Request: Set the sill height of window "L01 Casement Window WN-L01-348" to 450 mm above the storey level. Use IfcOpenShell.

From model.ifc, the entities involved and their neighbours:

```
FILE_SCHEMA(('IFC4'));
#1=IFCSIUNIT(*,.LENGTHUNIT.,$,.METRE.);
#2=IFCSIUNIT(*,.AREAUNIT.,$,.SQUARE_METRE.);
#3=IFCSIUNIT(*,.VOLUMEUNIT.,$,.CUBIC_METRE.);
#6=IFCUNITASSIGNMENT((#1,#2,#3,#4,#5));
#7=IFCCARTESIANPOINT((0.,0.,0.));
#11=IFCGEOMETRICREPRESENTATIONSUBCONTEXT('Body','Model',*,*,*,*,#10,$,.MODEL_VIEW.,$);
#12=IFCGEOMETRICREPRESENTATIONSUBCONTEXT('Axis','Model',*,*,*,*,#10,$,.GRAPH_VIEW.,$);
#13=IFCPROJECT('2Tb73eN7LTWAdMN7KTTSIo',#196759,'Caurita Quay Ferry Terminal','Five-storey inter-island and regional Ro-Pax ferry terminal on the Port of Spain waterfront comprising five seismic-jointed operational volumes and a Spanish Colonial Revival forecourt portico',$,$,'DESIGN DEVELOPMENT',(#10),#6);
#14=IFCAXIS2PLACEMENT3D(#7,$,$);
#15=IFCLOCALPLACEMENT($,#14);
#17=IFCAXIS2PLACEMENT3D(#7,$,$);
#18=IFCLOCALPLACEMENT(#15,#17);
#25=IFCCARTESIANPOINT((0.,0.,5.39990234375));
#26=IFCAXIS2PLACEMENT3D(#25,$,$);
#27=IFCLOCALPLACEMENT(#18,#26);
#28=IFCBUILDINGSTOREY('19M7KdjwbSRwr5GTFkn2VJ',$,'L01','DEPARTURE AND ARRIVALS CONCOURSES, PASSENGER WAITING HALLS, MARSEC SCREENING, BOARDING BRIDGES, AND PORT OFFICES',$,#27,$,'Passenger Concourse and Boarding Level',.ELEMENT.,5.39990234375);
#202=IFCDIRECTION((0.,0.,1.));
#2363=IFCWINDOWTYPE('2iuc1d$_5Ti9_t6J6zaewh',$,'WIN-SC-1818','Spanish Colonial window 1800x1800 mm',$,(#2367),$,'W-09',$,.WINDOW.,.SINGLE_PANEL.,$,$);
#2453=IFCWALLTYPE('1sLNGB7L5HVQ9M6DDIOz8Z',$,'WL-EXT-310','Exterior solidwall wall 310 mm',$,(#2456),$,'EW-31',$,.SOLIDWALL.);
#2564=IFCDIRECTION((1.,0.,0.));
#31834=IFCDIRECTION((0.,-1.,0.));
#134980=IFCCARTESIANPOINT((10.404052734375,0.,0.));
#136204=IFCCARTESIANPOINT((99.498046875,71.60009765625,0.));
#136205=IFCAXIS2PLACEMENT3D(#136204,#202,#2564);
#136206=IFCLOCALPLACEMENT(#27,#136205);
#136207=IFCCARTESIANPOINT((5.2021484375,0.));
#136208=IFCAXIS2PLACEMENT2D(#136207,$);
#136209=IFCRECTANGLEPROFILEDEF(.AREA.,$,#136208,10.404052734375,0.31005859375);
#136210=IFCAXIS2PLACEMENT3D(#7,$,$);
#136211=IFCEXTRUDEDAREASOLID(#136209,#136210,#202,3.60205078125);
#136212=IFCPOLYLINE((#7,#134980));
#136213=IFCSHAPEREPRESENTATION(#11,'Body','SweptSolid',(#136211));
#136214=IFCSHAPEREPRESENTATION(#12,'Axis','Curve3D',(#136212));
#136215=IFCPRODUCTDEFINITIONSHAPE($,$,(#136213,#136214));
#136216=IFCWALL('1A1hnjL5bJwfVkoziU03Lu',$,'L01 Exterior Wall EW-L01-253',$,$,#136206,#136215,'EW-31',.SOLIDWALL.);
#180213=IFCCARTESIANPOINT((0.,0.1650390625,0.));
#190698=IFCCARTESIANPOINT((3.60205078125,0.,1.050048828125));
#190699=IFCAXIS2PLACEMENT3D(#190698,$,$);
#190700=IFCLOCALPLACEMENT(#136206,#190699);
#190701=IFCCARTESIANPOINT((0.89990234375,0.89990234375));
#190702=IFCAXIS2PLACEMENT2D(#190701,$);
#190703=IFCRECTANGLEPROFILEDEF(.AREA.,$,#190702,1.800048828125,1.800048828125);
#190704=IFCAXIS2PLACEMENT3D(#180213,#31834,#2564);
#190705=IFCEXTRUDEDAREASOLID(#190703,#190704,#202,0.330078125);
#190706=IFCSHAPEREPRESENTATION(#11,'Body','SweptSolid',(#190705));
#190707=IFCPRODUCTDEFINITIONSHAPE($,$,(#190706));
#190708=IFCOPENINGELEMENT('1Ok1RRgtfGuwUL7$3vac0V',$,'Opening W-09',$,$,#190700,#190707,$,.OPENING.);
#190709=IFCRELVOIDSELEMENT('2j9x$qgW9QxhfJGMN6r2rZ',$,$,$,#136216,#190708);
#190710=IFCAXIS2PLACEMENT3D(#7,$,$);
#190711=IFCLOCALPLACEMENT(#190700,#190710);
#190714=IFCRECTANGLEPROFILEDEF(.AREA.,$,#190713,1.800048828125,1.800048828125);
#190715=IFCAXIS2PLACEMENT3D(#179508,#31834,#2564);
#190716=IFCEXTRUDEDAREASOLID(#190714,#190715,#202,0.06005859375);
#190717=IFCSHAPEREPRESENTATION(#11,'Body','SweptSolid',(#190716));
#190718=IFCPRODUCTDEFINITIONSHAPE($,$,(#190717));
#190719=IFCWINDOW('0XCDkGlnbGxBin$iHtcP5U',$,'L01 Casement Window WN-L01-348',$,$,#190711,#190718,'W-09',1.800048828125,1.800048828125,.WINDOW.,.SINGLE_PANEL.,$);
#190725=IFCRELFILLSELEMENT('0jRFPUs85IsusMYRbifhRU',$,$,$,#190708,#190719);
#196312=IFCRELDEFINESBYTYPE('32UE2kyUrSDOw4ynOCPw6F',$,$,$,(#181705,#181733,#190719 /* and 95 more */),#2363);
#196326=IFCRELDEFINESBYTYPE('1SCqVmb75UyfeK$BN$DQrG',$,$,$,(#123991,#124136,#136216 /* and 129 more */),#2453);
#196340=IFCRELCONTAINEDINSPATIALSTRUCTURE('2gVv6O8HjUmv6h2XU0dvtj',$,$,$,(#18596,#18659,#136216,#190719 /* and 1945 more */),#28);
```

```python
import numpy as np
import ifcopenshell
import ifcopenshell.api.geometry
import ifcopenshell.geom
import ifcopenshell.util.element
import ifcopenshell.util.placement
import ifcopenshell.util.shape
import ifcopenshell.util.unit

model = ifcopenshell.open("model.ifc")
unit_scale = ifcopenshell.util.unit.calculate_unit_scale(model)

window = model.by_guid("0XCDkGlnbGxBin$iHtcP5U")
opening = window.FillsVoids[0].RelatingOpeningElement
storey = ifcopenshell.util.element.get_container(window, ifc_class="IfcBuildingStorey")
level = ifcopenshell.util.placement.get_local_placement(storey.ObjectPlacement)[2, 3]

# The opening's origin need not be at the sill, so measure its lowest point.
shape = ifcopenshell.geom.create_shape(ifcopenshell.geom.settings(), opening)
bottom = ifcopenshell.util.shape.get_shape_bottom_elevation(shape, shape.geometry) / unit_scale
dz = level + 0.45 / unit_scale - bottom

shift = np.array([0.0, 0.0, dz])
# The window is placed relative to its opening, so it follows when the opening moves.
matrix = ifcopenshell.util.placement.get_local_placement(opening.ObjectPlacement)
matrix[:3, 3] += shift
ifcopenshell.api.geometry.edit_object_placement(
    model, product=opening, matrix=matrix, is_si=False, should_transform_children=True
)

print(f"moved by {dz * unit_scale:+.3f} m")

model.write("model_edited.ifc")
```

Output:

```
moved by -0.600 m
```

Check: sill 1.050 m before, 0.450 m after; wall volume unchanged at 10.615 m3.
